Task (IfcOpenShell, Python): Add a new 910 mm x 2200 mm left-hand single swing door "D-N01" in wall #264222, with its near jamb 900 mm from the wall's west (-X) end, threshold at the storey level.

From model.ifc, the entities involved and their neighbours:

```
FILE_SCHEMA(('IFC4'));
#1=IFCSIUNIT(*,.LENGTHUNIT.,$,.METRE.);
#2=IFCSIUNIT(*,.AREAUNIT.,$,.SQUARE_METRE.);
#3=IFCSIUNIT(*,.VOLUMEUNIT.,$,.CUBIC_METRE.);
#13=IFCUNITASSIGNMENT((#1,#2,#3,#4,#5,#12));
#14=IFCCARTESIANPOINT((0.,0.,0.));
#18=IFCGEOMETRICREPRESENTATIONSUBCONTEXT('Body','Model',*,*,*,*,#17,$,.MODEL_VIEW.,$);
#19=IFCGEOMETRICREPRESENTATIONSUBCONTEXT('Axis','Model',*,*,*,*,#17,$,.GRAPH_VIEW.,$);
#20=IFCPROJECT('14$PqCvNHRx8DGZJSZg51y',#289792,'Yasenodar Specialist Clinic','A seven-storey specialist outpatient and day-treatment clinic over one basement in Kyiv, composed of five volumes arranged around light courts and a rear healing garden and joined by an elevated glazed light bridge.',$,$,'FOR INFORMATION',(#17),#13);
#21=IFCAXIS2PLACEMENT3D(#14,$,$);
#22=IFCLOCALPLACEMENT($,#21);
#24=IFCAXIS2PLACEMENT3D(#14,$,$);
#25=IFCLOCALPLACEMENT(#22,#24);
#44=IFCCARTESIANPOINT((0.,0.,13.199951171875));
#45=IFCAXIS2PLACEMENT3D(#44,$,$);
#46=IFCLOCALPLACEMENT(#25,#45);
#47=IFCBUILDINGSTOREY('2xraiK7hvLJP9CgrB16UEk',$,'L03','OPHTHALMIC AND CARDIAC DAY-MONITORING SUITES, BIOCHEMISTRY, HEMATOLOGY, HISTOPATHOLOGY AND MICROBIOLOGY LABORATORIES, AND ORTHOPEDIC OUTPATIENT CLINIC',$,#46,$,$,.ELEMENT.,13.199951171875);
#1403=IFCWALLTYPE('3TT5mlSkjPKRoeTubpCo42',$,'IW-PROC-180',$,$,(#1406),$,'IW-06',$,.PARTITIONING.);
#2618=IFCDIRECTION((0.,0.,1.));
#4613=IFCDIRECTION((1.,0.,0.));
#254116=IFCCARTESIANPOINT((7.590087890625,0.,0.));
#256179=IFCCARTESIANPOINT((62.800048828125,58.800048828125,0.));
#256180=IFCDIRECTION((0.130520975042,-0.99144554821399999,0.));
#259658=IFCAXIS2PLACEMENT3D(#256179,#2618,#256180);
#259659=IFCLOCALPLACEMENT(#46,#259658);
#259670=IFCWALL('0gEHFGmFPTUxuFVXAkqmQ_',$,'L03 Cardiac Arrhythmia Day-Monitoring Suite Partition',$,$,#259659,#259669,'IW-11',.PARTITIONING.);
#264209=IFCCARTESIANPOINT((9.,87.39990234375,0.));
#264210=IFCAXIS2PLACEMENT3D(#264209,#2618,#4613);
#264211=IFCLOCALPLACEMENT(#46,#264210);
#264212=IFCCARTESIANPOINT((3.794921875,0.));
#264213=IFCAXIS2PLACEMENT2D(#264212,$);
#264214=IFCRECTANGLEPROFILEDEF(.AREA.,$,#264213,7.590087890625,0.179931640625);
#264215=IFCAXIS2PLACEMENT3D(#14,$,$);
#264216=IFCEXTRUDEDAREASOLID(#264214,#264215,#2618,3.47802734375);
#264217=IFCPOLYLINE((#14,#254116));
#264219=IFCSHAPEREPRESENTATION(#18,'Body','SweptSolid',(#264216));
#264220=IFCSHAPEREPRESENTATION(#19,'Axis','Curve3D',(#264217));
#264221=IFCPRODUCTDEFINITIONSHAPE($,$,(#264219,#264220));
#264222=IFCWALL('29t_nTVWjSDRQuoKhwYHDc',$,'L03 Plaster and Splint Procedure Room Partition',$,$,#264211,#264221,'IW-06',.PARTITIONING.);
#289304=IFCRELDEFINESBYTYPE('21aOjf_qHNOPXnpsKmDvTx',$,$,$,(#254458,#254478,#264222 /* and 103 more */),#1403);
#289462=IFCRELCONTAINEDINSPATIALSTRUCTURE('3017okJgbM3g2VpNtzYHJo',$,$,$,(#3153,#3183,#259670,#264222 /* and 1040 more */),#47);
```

```python
import numpy as np
import ifcopenshell
import ifcopenshell.api.feature
import ifcopenshell.api.geometry
import ifcopenshell.api.root
import ifcopenshell.api.spatial
import ifcopenshell.geom
import ifcopenshell.util.element
import ifcopenshell.util.placement
import ifcopenshell.util.representation
import ifcopenshell.util.shape
import ifcopenshell.util.unit

model = ifcopenshell.open("model.ifc")
unit_scale = ifcopenshell.util.unit.calculate_unit_scale(model)
settings = ifcopenshell.geom.settings()


def volume(element):
    """Net volume in cubic metres, openings subtracted."""
    shape = ifcopenshell.geom.create_shape(settings, element)
    return ifcopenshell.util.shape.get_volume(shape.geometry)


wall = model.by_id(264222)
storey = ifcopenshell.util.element.get_container(wall, ifc_class="IfcBuildingStorey")
context = ifcopenshell.util.representation.get_context(model, "Model", "Body", "MODEL_VIEW")
before = volume(wall)

width, height, from_end, sill = 0.91, 2.2, 0.9, 0.0  # metres

# The wall runs along its own X axis, and the end named is its -X end.
wall_shape = ifcopenshell.geom.create_shape(settings, wall)
x, y, z = ifcopenshell.util.shape.get_vertices(wall_shape.geometry).T
start = x.min() + from_end
face, thickness = float(y.min()), float(y.max() - y.min())
wall_matrix = ifcopenshell.util.placement.get_local_placement(wall.ObjectPlacement)
level = ifcopenshell.util.placement.get_local_placement(storey.ObjectPlacement)[2, 3]


def in_wall(x, y):
    """Placement at x, y metres in the wall's axes, at sill height."""
    matrix = wall_matrix.copy()
    matrix[:, 3] = wall_matrix @ np.array([x / unit_scale, y / unit_scale, 0.0, 1.0])
    matrix[2, 3] = level + sill / unit_scale
    return matrix


# Opening: a box that overshoots both wall faces by 50 mm.
opening = ifcopenshell.api.root.create_entity(model, ifc_class="IfcOpeningElement", predefined_type="OPENING")
box = ifcopenshell.api.geometry.add_wall_representation(
    model, context=context, length=width, height=height, thickness=thickness + 0.1
)
ifcopenshell.api.geometry.assign_representation(model, product=opening, representation=box)
ifcopenshell.api.geometry.edit_object_placement(model, product=opening, matrix=in_wall(start, face - 0.05), is_si=False)
ifcopenshell.api.feature.add_feature(model, feature=opening, element=wall)

door = ifcopenshell.api.root.create_entity(model, ifc_class="IfcDoor", name="D-N01", predefined_type="DOOR")
door.OverallWidth, door.OverallHeight = width / unit_scale, height / unit_scale
door.OperationType = "SINGLE_SWING_LEFT"
body = ifcopenshell.api.geometry.add_door_representation(
    model,
    context=context,
    overall_width=door.OverallWidth,
    overall_height=door.OverallHeight,
    operation_type="SINGLE_SWING_LEFT",
    lining_properties={"LiningDepth": thickness / unit_scale, "ThresholdDepth": thickness / unit_scale},
)
ifcopenshell.api.geometry.assign_representation(model, product=door, representation=body)
ifcopenshell.api.spatial.assign_container(model, products=[door], relating_structure=storey)
ifcopenshell.api.feature.add_filling(model, opening=opening, element=door)

# The lining spans the wall, so the door starts at the wall face.
ifcopenshell.api.geometry.edit_object_placement(model, product=door, matrix=in_wall(start, face), is_si=False)

after = volume(wall)

print(f"wall volume {before:.3f} -> {after:.3f} m3")

model.write("model_edited.ifc")
```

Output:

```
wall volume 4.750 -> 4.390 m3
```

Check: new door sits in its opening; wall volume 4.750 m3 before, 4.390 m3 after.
